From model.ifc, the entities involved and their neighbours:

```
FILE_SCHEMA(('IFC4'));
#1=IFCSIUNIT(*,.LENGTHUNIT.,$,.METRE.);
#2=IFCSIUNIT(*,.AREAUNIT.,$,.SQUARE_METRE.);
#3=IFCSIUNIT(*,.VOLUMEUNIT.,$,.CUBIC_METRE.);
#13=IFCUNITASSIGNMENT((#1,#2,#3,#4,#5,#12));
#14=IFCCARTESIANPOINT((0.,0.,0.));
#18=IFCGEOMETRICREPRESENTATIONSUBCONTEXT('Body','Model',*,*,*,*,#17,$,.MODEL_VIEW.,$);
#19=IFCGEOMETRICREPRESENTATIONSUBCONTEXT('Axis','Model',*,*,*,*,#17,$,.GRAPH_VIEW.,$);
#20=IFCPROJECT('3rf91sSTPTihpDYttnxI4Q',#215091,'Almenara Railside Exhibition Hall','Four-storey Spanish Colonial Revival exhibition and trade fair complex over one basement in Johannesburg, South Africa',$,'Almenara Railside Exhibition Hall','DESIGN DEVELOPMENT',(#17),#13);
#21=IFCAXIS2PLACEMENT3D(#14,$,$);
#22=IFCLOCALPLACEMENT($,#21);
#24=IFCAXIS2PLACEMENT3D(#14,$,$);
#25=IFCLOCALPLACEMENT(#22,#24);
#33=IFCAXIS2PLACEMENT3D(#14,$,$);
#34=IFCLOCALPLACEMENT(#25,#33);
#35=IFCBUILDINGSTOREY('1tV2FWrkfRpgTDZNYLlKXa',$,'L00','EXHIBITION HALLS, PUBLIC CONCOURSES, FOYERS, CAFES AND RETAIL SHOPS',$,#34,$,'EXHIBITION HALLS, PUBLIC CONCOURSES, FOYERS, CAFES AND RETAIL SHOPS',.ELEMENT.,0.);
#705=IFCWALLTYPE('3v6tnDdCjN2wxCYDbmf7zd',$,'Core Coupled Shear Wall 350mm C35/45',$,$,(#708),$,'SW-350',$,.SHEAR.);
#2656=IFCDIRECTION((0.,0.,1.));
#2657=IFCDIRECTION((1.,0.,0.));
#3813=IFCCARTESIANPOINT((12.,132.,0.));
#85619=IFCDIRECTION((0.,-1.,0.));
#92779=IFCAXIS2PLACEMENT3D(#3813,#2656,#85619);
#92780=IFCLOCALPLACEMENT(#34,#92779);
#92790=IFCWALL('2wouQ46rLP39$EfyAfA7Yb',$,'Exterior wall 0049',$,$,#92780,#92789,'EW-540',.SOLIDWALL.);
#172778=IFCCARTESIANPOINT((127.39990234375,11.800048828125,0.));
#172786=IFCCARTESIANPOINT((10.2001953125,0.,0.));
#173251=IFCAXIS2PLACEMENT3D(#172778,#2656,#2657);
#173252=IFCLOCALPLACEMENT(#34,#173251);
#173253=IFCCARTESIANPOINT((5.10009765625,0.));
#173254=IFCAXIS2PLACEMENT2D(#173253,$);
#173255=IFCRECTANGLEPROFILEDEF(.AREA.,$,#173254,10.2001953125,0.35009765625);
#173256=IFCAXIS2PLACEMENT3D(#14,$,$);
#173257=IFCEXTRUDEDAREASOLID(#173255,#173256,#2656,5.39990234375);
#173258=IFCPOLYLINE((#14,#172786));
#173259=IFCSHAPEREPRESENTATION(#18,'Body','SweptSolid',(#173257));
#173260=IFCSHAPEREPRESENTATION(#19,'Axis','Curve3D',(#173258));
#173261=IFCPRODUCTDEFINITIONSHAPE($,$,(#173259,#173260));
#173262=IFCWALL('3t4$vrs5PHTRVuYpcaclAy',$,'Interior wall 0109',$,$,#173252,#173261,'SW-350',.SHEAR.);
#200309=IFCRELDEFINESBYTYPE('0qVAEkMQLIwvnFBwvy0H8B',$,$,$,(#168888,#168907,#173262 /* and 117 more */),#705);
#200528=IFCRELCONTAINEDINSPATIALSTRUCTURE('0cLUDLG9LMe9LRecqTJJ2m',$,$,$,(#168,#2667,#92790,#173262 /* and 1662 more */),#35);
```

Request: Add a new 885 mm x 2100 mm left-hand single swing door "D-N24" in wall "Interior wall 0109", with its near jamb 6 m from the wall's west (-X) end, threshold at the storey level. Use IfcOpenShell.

```python
import numpy as np
import ifcopenshell
import ifcopenshell.api.feature
import ifcopenshell.api.geometry
import ifcopenshell.api.root
import ifcopenshell.api.spatial
import ifcopenshell.geom
import ifcopenshell.util.element
import ifcopenshell.util.placement
import ifcopenshell.util.representation
import ifcopenshell.util.shape
import ifcopenshell.util.unit

model = ifcopenshell.open("model.ifc")
unit_scale = ifcopenshell.util.unit.calculate_unit_scale(model)
settings = ifcopenshell.geom.settings()


def volume(element):
    """Net volume in cubic metres, openings subtracted."""
    shape = ifcopenshell.geom.create_shape(settings, element)
    return ifcopenshell.util.shape.get_volume(shape.geometry)


wall = model.by_guid("3t4$vrs5PHTRVuYpcaclAy")
storey = ifcopenshell.util.element.get_container(wall, ifc_class="IfcBuildingStorey")
context = ifcopenshell.util.representation.get_context(model, "Model", "Body", "MODEL_VIEW")
before = volume(wall)

width, height, from_end, sill = 0.885, 2.1, 6, 0.0  # metres

# The wall runs along its own X axis, and the end named is its -X end.
wall_shape = ifcopenshell.geom.create_shape(settings, wall)
x, y, z = ifcopenshell.util.shape.get_vertices(wall_shape.geometry).T
start = x.min() + from_end
face, thickness = float(y.min()), float(y.max() - y.min())
wall_matrix = ifcopenshell.util.placement.get_local_placement(wall.ObjectPlacement)
level = ifcopenshell.util.placement.get_local_placement(storey.ObjectPlacement)[2, 3]


def in_wall(x, y):
    """Placement at x, y metres in the wall's axes, at sill height."""
    matrix = wall_matrix.copy()
    matrix[:, 3] = wall_matrix @ np.array([x / unit_scale, y / unit_scale, 0.0, 1.0])
    matrix[2, 3] = level + sill / unit_scale
    return matrix


# Opening: a box that overshoots both wall faces by 50 mm.
opening = ifcopenshell.api.root.create_entity(model, ifc_class="IfcOpeningElement", predefined_type="OPENING")
box = ifcopenshell.api.geometry.add_wall_representation(
    model, context=context, length=width, height=height, thickness=thickness + 0.1
)
ifcopenshell.api.geometry.assign_representation(model, product=opening, representation=box)
ifcopenshell.api.geometry.edit_object_placement(model, product=opening, matrix=in_wall(start, face - 0.05), is_si=False)
ifcopenshell.api.feature.add_feature(model, feature=opening, element=wall)

door = ifcopenshell.api.root.create_entity(model, ifc_class="IfcDoor", name="D-N24", predefined_type="DOOR")
door.OverallWidth, door.OverallHeight = width / unit_scale, height / unit_scale
door.OperationType = "SINGLE_SWING_LEFT"
body = ifcopenshell.api.geometry.add_door_representation(
    model,
    context=context,
    overall_width=door.OverallWidth,
    overall_height=door.OverallHeight,
    operation_type="SINGLE_SWING_LEFT",
    lining_properties={"LiningDepth": thickness / unit_scale, "ThresholdDepth": thickness / unit_scale},
)
ifcopenshell.api.geometry.assign_representation(model, product=door, representation=body)
ifcopenshell.api.spatial.assign_container(model, products=[door], relating_structure=storey)
ifcopenshell.api.feature.add_filling(model, opening=opening, element=door)

# The lining spans the wall, so the door starts at the wall face.
ifcopenshell.api.geometry.edit_object_placement(model, product=door, matrix=in_wall(start, face), is_si=False)

after = volume(wall)

print(f"wall volume {before:.3f} -> {after:.3f} m3")

model.write("model-out.ifc")
```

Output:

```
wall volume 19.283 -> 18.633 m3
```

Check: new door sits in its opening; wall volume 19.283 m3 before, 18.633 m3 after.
